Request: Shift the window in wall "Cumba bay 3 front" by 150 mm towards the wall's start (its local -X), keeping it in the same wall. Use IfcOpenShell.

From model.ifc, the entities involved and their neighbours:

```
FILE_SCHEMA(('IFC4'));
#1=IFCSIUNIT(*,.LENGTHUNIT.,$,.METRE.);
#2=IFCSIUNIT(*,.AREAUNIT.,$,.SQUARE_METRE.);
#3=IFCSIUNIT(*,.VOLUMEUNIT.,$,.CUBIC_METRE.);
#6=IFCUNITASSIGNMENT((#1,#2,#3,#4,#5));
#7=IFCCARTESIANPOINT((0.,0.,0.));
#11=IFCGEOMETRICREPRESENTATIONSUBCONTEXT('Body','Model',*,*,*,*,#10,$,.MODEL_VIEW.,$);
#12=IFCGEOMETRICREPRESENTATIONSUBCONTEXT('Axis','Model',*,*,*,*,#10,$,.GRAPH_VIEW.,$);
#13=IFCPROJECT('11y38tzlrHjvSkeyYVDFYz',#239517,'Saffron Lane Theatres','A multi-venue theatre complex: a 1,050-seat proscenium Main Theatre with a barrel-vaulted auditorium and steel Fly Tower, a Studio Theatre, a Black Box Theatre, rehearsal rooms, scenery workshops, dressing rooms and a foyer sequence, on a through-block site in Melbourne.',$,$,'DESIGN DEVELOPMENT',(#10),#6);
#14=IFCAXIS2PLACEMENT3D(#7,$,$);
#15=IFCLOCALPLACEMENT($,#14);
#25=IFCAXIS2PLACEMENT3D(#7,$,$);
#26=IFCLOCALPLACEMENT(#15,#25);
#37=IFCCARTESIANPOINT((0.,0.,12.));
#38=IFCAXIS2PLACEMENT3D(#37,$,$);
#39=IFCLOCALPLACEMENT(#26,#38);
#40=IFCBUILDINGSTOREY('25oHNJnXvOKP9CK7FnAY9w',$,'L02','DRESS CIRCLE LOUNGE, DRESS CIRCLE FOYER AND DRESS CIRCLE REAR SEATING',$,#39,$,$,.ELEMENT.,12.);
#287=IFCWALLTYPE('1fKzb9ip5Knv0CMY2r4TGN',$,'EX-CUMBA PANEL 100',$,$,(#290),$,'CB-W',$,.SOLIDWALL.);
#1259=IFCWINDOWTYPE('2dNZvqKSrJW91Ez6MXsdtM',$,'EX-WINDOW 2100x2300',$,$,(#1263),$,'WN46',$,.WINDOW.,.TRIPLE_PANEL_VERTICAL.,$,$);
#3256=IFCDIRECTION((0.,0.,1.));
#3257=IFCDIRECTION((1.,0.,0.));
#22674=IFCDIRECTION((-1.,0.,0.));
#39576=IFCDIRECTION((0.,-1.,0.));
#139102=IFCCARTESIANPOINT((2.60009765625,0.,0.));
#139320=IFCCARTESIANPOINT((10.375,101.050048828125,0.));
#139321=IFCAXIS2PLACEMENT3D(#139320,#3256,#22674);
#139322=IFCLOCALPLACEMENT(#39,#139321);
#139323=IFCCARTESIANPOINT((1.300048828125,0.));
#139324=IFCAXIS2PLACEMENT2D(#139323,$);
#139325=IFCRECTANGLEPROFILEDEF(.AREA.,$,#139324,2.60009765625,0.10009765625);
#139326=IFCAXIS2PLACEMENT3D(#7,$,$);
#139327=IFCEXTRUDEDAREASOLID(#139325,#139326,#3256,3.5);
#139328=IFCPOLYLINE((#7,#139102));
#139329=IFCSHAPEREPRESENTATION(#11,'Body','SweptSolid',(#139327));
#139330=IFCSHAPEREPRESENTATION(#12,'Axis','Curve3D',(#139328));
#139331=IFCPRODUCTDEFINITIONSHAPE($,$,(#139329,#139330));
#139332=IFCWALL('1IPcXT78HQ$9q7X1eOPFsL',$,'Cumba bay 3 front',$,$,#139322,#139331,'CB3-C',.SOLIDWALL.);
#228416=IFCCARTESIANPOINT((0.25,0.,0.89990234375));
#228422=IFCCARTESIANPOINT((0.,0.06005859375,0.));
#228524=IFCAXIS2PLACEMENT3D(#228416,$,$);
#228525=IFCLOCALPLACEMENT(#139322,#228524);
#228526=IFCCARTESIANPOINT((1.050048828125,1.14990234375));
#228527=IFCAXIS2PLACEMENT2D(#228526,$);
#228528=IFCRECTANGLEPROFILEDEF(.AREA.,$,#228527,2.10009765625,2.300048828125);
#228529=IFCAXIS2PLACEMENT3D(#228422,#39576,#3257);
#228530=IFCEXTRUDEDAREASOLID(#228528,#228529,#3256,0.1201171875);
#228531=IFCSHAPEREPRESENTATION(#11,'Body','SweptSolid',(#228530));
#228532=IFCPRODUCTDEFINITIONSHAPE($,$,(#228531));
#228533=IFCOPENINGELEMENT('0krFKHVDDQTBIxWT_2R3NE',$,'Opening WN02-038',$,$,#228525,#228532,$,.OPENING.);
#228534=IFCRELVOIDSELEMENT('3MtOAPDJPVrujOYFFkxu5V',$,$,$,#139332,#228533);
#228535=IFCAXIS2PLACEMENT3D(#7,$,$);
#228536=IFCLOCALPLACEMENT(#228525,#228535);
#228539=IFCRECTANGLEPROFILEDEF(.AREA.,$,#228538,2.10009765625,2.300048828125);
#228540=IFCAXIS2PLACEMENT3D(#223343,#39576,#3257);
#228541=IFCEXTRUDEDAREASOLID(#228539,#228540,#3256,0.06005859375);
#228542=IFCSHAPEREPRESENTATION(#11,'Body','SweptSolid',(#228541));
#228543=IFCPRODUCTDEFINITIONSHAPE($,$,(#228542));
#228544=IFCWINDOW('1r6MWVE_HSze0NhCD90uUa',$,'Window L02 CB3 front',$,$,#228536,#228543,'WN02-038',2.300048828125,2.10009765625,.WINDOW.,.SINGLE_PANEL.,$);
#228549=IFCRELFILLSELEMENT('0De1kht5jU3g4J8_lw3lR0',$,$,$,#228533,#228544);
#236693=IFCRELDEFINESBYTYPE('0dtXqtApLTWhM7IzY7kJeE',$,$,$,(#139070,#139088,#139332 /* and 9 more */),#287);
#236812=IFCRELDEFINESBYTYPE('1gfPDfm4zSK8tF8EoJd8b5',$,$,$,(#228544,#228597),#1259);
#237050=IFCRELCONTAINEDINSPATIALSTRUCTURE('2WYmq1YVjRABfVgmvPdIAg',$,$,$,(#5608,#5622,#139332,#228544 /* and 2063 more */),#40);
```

```python
import ifcopenshell
import ifcopenshell.api.geometry
import ifcopenshell.util.placement

model = ifcopenshell.open("model.ifc")

window = model.by_guid("1r6MWVE_HSze0NhCD90uUa")
opening = window.FillsVoids[0].RelatingOpeningElement
wall = opening.VoidsElements[0].RelatingBuildingElement

wall_matrix = ifcopenshell.util.placement.get_local_placement(wall.ObjectPlacement)
shift = wall_matrix[:3, 0] * -0.15
before = ifcopenshell.util.placement.get_local_placement(window.ObjectPlacement)[:3, 3].copy()

# The window is placed relative to its opening, so it follows when the opening moves.
matrix = ifcopenshell.util.placement.get_local_placement(opening.ObjectPlacement)
matrix[:3, 3] += shift
ifcopenshell.api.geometry.edit_object_placement(
    model, product=opening, matrix=matrix, is_si=False, should_transform_children=True
)

after = ifcopenshell.util.placement.get_local_placement(window.ObjectPlacement)[:3, 3]
print("window moved by", (after - before).round(3) + 0.0)

model.write("model-out.ifc")
```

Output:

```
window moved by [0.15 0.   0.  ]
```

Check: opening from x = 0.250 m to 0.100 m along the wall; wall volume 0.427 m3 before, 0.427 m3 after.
